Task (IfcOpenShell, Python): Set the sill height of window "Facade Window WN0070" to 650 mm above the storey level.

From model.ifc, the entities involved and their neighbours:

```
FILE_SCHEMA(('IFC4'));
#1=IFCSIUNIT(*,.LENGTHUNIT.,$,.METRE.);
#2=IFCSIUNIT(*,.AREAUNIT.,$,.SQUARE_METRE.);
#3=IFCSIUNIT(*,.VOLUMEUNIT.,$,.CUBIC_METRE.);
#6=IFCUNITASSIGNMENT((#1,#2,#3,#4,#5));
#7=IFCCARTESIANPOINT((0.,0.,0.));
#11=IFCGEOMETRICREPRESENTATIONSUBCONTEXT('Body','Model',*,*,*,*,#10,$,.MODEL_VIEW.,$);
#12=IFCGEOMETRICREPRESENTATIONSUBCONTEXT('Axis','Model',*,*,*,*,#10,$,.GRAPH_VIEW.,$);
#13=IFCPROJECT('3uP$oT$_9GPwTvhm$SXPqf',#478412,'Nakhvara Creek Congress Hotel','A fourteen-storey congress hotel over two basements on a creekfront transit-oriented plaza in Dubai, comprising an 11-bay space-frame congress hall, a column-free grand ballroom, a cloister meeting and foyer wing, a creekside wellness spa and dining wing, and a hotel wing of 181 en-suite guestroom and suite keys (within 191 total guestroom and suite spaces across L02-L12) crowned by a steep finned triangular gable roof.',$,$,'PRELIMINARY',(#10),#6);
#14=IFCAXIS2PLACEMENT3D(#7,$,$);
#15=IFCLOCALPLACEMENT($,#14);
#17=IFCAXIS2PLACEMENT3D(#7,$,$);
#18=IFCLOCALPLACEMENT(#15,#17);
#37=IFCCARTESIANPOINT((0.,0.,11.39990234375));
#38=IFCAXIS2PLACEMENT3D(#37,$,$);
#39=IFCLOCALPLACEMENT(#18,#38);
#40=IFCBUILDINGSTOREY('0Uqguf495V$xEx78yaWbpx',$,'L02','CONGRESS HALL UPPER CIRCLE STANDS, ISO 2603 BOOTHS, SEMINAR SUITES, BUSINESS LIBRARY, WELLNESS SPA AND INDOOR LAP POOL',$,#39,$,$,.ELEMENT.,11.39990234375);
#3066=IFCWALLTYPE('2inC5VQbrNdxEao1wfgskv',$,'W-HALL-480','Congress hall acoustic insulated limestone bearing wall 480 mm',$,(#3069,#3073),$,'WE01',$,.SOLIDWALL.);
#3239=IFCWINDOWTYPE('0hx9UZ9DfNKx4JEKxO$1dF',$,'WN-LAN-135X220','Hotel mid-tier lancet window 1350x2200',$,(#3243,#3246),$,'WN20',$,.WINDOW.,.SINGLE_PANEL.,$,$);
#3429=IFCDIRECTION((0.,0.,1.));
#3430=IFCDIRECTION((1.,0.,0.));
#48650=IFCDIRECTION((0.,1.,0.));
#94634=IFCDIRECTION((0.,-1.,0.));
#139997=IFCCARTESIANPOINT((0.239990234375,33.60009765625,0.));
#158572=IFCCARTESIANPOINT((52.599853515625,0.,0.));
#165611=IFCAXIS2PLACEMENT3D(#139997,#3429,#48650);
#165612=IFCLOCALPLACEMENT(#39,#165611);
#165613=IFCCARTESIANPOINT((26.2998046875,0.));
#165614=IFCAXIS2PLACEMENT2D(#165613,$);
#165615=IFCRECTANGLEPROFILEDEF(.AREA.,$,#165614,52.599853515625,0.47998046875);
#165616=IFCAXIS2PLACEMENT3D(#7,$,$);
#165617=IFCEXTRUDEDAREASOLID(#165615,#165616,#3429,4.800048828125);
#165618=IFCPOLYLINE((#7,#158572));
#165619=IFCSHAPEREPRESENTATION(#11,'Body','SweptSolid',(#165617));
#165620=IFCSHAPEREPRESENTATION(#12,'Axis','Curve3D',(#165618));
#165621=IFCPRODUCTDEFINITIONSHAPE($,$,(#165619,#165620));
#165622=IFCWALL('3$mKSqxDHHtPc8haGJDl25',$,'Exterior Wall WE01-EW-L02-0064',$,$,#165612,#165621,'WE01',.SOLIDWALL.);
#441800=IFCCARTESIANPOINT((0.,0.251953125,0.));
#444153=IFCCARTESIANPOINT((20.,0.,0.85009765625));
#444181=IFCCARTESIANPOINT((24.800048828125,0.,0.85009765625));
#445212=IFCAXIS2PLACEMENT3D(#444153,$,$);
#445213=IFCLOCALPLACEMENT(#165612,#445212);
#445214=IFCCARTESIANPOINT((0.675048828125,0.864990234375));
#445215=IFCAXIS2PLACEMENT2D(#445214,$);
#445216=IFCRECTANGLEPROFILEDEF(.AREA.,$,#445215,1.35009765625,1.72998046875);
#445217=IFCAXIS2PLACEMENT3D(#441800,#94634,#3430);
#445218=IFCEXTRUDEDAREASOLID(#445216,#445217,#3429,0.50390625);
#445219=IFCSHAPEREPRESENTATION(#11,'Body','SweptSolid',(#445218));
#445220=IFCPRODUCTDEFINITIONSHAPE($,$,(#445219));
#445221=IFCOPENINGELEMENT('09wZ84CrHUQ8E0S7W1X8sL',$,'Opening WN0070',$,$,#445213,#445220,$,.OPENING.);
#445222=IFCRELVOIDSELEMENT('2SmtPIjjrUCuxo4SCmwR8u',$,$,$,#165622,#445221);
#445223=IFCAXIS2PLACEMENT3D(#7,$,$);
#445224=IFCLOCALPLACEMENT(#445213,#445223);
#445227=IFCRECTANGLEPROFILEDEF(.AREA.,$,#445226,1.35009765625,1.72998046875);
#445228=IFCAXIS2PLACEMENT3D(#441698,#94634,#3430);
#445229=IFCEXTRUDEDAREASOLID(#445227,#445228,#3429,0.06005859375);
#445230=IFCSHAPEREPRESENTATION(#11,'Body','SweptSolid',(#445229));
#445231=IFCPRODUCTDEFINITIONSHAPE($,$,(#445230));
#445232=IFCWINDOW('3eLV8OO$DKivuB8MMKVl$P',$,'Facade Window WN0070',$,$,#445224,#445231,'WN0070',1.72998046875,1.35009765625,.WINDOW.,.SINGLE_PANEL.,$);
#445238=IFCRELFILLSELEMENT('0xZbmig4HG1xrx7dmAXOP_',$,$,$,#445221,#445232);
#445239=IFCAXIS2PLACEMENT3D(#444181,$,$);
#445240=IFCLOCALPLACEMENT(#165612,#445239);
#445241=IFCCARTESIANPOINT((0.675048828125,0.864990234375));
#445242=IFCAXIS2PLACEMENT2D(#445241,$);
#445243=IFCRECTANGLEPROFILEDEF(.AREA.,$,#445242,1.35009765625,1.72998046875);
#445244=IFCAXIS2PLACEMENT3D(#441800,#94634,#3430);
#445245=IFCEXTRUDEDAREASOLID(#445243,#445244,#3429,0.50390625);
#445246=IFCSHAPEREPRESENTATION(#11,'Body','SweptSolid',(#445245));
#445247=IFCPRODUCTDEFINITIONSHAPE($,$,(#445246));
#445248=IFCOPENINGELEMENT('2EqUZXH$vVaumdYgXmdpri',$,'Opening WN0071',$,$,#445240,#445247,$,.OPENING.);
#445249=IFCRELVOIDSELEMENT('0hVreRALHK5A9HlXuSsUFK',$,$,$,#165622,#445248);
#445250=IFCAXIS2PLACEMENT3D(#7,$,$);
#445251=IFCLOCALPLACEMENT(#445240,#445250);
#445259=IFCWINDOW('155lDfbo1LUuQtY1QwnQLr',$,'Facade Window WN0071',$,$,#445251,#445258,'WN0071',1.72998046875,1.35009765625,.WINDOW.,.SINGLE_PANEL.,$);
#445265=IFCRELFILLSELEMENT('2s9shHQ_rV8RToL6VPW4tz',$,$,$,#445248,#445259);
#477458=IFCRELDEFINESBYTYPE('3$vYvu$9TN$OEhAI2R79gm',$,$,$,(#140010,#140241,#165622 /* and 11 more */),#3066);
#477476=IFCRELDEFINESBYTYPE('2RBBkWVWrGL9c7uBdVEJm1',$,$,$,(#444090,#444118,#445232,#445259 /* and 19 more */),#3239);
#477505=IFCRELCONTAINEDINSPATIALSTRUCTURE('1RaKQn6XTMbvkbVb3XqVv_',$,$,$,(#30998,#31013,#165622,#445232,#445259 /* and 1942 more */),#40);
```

```python
import numpy as np
import ifcopenshell
import ifcopenshell.api.geometry
import ifcopenshell.geom
import ifcopenshell.util.element
import ifcopenshell.util.placement
import ifcopenshell.util.shape
import ifcopenshell.util.unit

model = ifcopenshell.open("model.ifc")
unit_scale = ifcopenshell.util.unit.calculate_unit_scale(model)

window = model.by_id(445232)
opening = window.FillsVoids[0].RelatingOpeningElement
storey = ifcopenshell.util.element.get_container(window, ifc_class="IfcBuildingStorey")
level = ifcopenshell.util.placement.get_local_placement(storey.ObjectPlacement)[2, 3]

# The opening's origin need not be at the sill, so measure its lowest point.
shape = ifcopenshell.geom.create_shape(ifcopenshell.geom.settings(), opening)
bottom = ifcopenshell.util.shape.get_shape_bottom_elevation(shape, shape.geometry) / unit_scale
dz = level + 0.65 / unit_scale - bottom

shift = np.array([0.0, 0.0, dz])
# The window is placed relative to its opening, so it follows when the opening moves.
matrix = ifcopenshell.util.placement.get_local_placement(opening.ObjectPlacement)
matrix[:3, 3] += shift
ifcopenshell.api.geometry.edit_object_placement(
    model, product=opening, matrix=matrix, is_si=False, should_transform_children=True
)

print(f"moved by {dz * unit_scale:+.3f} m")

model.write("model_edited.ifc")
```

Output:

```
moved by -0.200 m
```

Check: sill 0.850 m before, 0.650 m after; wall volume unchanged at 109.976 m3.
